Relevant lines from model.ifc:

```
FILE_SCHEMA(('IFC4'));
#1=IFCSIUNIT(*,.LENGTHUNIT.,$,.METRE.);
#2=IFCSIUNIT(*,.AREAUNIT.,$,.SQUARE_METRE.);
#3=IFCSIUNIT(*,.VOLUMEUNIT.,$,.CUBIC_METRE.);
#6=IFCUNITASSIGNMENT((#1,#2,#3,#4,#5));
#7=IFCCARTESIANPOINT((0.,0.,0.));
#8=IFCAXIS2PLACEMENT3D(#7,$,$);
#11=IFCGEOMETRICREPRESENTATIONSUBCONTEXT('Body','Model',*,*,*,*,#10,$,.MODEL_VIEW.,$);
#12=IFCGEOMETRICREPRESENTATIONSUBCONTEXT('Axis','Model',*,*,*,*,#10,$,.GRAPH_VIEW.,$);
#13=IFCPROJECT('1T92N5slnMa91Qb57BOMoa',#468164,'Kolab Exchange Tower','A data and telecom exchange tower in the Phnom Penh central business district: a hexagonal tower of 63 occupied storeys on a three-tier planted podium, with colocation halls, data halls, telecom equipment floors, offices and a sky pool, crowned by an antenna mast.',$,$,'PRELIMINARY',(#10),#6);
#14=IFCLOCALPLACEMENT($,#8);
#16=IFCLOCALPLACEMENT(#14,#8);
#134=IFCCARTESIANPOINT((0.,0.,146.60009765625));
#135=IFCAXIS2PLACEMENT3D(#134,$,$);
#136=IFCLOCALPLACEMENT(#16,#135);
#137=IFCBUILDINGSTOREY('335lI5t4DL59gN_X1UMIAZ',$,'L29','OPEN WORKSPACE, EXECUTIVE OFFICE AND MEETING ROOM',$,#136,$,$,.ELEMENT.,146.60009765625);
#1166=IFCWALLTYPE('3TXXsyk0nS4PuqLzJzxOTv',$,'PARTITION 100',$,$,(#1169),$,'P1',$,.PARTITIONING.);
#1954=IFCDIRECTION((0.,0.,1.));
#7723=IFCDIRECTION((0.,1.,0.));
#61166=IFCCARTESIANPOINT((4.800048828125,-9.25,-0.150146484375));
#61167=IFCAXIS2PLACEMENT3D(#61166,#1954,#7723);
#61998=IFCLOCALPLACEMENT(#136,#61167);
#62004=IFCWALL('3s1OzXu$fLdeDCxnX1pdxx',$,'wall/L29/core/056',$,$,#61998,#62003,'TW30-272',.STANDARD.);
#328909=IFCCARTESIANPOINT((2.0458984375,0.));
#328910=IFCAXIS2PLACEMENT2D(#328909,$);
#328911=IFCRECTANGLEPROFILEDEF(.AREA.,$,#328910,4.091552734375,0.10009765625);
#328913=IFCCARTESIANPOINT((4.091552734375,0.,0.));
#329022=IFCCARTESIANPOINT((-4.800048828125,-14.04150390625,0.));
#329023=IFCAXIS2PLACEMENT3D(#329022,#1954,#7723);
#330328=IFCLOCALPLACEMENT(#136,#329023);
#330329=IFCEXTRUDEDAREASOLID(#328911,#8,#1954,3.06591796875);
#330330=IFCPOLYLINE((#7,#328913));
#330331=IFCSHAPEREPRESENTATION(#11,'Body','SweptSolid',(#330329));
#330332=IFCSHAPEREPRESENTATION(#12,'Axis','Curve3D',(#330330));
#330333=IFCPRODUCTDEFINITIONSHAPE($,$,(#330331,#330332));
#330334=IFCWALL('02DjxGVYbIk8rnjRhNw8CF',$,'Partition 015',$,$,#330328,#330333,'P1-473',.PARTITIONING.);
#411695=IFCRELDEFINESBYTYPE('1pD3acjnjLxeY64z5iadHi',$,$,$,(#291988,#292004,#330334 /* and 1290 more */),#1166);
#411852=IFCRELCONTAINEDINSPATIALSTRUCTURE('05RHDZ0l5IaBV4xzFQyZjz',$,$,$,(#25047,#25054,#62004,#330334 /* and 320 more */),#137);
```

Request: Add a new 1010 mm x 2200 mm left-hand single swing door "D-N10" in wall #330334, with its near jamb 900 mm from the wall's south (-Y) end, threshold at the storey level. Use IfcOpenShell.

```python
import numpy as np
import ifcopenshell
import ifcopenshell.api.feature
import ifcopenshell.api.geometry
import ifcopenshell.api.root
import ifcopenshell.api.spatial
import ifcopenshell.geom
import ifcopenshell.util.element
import ifcopenshell.util.placement
import ifcopenshell.util.representation
import ifcopenshell.util.shape
import ifcopenshell.util.unit

model = ifcopenshell.open("model.ifc")
unit_scale = ifcopenshell.util.unit.calculate_unit_scale(model)
settings = ifcopenshell.geom.settings()


def volume(element):
    """Net volume in cubic metres, openings subtracted."""
    shape = ifcopenshell.geom.create_shape(settings, element)
    return ifcopenshell.util.shape.get_volume(shape.geometry)


wall = model.by_guid("02DjxGVYbIk8rnjRhNw8CF")
storey = ifcopenshell.util.element.get_container(wall, ifc_class="IfcBuildingStorey")
context = ifcopenshell.util.representation.get_context(model, "Model", "Body", "MODEL_VIEW")
before = volume(wall)

width, height, from_end, sill = 1.01, 2.2, 0.9, 0.0  # metres

# The wall runs along its own X axis, and the end named is its -X end.
wall_shape = ifcopenshell.geom.create_shape(settings, wall)
x, y, z = ifcopenshell.util.shape.get_vertices(wall_shape.geometry).T
start = x.min() + from_end
face, thickness = float(y.min()), float(y.max() - y.min())
wall_matrix = ifcopenshell.util.placement.get_local_placement(wall.ObjectPlacement)
level = ifcopenshell.util.placement.get_local_placement(storey.ObjectPlacement)[2, 3]


def in_wall(x, y):
    """Placement at x, y metres in the wall's axes, at sill height."""
    matrix = wall_matrix.copy()
    matrix[:, 3] = wall_matrix @ np.array([x / unit_scale, y / unit_scale, 0.0, 1.0])
    matrix[2, 3] = level + sill / unit_scale
    return matrix


# Opening: a box that overshoots both wall faces by 50 mm.
opening = ifcopenshell.api.root.create_entity(model, ifc_class="IfcOpeningElement", predefined_type="OPENING")
box = ifcopenshell.api.geometry.add_wall_representation(
    model, context=context, length=width, height=height, thickness=thickness + 0.1
)
ifcopenshell.api.geometry.assign_representation(model, product=opening, representation=box)
ifcopenshell.api.geometry.edit_object_placement(model, product=opening, matrix=in_wall(start, face - 0.05), is_si=False)
ifcopenshell.api.feature.add_feature(model, feature=opening, element=wall)

door = ifcopenshell.api.root.create_entity(model, ifc_class="IfcDoor", name="D-N10", predefined_type="DOOR")
door.OverallWidth, door.OverallHeight = width / unit_scale, height / unit_scale
door.OperationType = "SINGLE_SWING_LEFT"
body = ifcopenshell.api.geometry.add_door_representation(
    model,
    context=context,
    overall_width=door.OverallWidth,
    overall_height=door.OverallHeight,
    operation_type="SINGLE_SWING_LEFT",
    lining_properties={"LiningDepth": thickness / unit_scale, "ThresholdDepth": thickness / unit_scale},
)
ifcopenshell.api.geometry.assign_representation(model, product=door, representation=body)
ifcopenshell.api.spatial.assign_container(model, products=[door], relating_structure=storey)
ifcopenshell.api.feature.add_filling(model, opening=opening, element=door)

# The lining spans the wall, so the door starts at the wall face.
ifcopenshell.api.geometry.edit_object_placement(model, product=door, matrix=in_wall(start, face), is_si=False)

after = volume(wall)

print(f"wall volume {before:.3f} -> {after:.3f} m3")

model.write("model_updated.ifc")
```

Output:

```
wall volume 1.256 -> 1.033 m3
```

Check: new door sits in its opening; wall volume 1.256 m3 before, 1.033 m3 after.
